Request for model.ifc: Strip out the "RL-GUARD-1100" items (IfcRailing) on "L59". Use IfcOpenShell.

First a look at what the model holds.

```python
import ifcopenshell
import ifcopenshell.util.element

model = ifcopenshell.open("model.ifc")
print(model.schema)
storey = next(s for s in model.by_type("IfcBuildingStorey") if s.Name == "L59")
railings = [e for e in ifcopenshell.util.element.get_decomposition(storey) if e.is_a("IfcRailing")]
seen = {}
for e in railings:
    element_type = ifcopenshell.util.element.get_type(e)
    name = element_type.Name if element_type not in (None, e) else None
    seen[name] = seen.get(name, 0) + 1
for name, count in sorted(seen.items(), key=str):
    print(count, "x", name)
```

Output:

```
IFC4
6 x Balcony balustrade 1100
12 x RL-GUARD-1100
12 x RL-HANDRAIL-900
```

```python
import ifcopenshell
import ifcopenshell.api.root
import ifcopenshell.util.element

model = ifcopenshell.open("model.ifc")

storey = next(s for s in model.by_type("IfcBuildingStorey") if s.Name == "L59")
railings = [e for e in ifcopenshell.util.element.get_decomposition(storey) if e.is_a("IfcRailing")]
targets = [e for e in railings if (t := ifcopenshell.util.element.get_type(e)) not in (None, e) and t.Name == "RL-GUARD-1100"]

for e in targets:
    ifcopenshell.api.root.remove_product(model, product=e)
print(len(targets), "removed")

model.write("model_updated.ifc")
```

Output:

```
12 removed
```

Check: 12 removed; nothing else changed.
